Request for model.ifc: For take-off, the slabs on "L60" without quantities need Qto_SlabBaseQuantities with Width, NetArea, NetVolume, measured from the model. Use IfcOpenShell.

First a look at what the model holds.

```python
import ifcopenshell
import ifcopenshell.util.element
import ifcopenshell.util.unit

model = ifcopenshell.open("model.ifc")
print(model.schema)
for unit_type in ("LENGTHUNIT", "AREAUNIT", "VOLUMEUNIT"):
    print(unit_type, ifcopenshell.util.unit.calculate_unit_scale(model, unit_type))
storey = next(s for s in model.by_type("IfcBuildingStorey") if s.Name == "L60")
slabs = [e for e in ifcopenshell.util.element.get_decomposition(storey) if e.is_a("IfcSlab")]
for e in sorted(slabs, key=lambda e: e.id()):
    print(e.id(), e.is_a(), e.Name, list(ifcopenshell.util.element.get_psets(e, qtos_only=True)), sep=" | ")
```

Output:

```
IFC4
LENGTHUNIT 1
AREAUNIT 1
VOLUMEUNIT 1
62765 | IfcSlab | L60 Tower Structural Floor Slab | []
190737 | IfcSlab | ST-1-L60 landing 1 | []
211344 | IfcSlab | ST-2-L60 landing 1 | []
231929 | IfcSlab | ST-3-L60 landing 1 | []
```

```python
import ifcopenshell
import ifcopenshell.api.pset
import ifcopenshell.geom
import ifcopenshell.util.element
import ifcopenshell.util.shape
import ifcopenshell.util.unit

model = ifcopenshell.open("model.ifc")
unit_scale = ifcopenshell.util.unit.calculate_unit_scale(model)
area_scale = ifcopenshell.util.unit.calculate_unit_scale(model, "AREAUNIT")
volume_scale = ifcopenshell.util.unit.calculate_unit_scale(model, "VOLUMEUNIT")
settings = ifcopenshell.geom.settings()

storey = next(s for s in model.by_type("IfcBuildingStorey") if s.Name == "L60")
slabs = [e for e in ifcopenshell.util.element.get_decomposition(storey) if e.is_a("IfcSlab")]

for e in sorted(slabs, key=lambda e: e.id()):
    if ifcopenshell.util.element.get_psets(e, qtos_only=True, should_inherit=False):
        continue
    # Geometry comes back in metres, in the element's own axes.
    shape = ifcopenshell.geom.create_shape(settings, e)
    values = {
        "Width": ifcopenshell.util.shape.get_z(shape.geometry) / unit_scale,
        "NetArea": ifcopenshell.util.shape.get_footprint_area(shape.geometry) / area_scale,
        "NetVolume": ifcopenshell.util.shape.get_volume(shape.geometry) / volume_scale,
    }
    qto = ifcopenshell.api.pset.add_qto(model, product=e, name="Qto_SlabBaseQuantities")
    ifcopenshell.api.pset.edit_qto(model, qto=qto, properties=values)
    print(e.id(), {k: round(v, 3) for k, v in values.items()})

model.write("model_edited.ifc")
```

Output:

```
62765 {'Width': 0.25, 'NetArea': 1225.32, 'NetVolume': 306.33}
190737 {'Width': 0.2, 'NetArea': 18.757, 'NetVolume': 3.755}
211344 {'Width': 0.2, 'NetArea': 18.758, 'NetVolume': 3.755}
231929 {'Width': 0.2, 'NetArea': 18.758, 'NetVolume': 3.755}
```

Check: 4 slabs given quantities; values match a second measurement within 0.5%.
